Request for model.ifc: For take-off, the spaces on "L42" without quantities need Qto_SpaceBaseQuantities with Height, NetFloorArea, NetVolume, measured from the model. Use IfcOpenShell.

First a look at what the model holds.

```python
import ifcopenshell
import ifcopenshell.util.element
import ifcopenshell.util.unit

model = ifcopenshell.open("model.ifc")
print(model.schema)
for unit_type in ("LENGTHUNIT", "AREAUNIT", "VOLUMEUNIT"):
    print(unit_type, ifcopenshell.util.unit.calculate_unit_scale(model, unit_type))
storey = next(s for s in model.by_type("IfcBuildingStorey") if s.Name == "L42")
spaces = [e for e in ifcopenshell.util.element.get_decomposition(storey) if e.is_a("IfcSpace")]
for e in sorted(spaces, key=lambda e: e.id()):
    print(e.id(), e.is_a(), e.Name, list(ifcopenshell.util.element.get_psets(e, qtos_only=True)), sep=" | ")
```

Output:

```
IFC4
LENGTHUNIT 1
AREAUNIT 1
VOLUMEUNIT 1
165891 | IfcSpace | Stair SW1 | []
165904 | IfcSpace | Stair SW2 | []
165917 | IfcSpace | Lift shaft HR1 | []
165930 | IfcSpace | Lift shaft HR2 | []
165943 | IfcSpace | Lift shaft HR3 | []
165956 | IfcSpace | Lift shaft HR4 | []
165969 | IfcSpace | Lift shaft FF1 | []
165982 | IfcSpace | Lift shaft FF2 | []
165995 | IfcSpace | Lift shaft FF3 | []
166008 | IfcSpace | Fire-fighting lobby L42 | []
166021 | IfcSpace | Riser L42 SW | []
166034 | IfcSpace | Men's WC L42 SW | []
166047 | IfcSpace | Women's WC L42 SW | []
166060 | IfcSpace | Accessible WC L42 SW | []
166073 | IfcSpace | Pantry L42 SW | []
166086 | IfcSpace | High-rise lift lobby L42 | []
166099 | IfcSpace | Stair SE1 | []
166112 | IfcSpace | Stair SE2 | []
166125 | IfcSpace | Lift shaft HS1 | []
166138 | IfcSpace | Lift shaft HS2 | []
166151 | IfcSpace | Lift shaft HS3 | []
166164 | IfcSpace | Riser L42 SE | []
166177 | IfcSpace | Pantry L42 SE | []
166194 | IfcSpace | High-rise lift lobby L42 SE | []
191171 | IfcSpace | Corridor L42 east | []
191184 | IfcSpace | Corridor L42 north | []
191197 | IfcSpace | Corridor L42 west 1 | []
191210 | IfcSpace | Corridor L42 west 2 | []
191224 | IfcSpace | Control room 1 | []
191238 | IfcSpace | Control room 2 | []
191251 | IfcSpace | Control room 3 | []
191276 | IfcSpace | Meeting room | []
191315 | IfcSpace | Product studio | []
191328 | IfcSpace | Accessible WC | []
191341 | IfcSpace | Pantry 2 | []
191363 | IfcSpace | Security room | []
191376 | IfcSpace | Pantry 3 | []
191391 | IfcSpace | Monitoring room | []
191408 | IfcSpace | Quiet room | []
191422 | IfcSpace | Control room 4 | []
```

```python
import ifcopenshell
import ifcopenshell.api.pset
import ifcopenshell.geom
import ifcopenshell.util.element
import ifcopenshell.util.shape
import ifcopenshell.util.unit

model = ifcopenshell.open("model.ifc")
unit_scale = ifcopenshell.util.unit.calculate_unit_scale(model)
area_scale = ifcopenshell.util.unit.calculate_unit_scale(model, "AREAUNIT")
volume_scale = ifcopenshell.util.unit.calculate_unit_scale(model, "VOLUMEUNIT")
settings = ifcopenshell.geom.settings()

storey = next(s for s in model.by_type("IfcBuildingStorey") if s.Name == "L42")
spaces = [e for e in ifcopenshell.util.element.get_decomposition(storey) if e.is_a("IfcSpace")]

for e in sorted(spaces, key=lambda e: e.id()):
    if ifcopenshell.util.element.get_psets(e, qtos_only=True, should_inherit=False):
        continue
    # Geometry comes back in metres, in the element's own axes.
    shape = ifcopenshell.geom.create_shape(settings, e)
    values = {
        "Height": ifcopenshell.util.shape.get_z(shape.geometry) / unit_scale,
        "NetFloorArea": ifcopenshell.util.shape.get_footprint_area(shape.geometry) / area_scale,
        "NetVolume": ifcopenshell.util.shape.get_volume(shape.geometry) / volume_scale,
    }
    qto = ifcopenshell.api.pset.add_qto(model, product=e, name="Qto_SpaceBaseQuantities")
    ifcopenshell.api.pset.edit_qto(model, qto=qto, properties=values)
    print(e.id(), {k: round(v, 3) for k, v in values.items()})

model.write("model_rev.ifc")
```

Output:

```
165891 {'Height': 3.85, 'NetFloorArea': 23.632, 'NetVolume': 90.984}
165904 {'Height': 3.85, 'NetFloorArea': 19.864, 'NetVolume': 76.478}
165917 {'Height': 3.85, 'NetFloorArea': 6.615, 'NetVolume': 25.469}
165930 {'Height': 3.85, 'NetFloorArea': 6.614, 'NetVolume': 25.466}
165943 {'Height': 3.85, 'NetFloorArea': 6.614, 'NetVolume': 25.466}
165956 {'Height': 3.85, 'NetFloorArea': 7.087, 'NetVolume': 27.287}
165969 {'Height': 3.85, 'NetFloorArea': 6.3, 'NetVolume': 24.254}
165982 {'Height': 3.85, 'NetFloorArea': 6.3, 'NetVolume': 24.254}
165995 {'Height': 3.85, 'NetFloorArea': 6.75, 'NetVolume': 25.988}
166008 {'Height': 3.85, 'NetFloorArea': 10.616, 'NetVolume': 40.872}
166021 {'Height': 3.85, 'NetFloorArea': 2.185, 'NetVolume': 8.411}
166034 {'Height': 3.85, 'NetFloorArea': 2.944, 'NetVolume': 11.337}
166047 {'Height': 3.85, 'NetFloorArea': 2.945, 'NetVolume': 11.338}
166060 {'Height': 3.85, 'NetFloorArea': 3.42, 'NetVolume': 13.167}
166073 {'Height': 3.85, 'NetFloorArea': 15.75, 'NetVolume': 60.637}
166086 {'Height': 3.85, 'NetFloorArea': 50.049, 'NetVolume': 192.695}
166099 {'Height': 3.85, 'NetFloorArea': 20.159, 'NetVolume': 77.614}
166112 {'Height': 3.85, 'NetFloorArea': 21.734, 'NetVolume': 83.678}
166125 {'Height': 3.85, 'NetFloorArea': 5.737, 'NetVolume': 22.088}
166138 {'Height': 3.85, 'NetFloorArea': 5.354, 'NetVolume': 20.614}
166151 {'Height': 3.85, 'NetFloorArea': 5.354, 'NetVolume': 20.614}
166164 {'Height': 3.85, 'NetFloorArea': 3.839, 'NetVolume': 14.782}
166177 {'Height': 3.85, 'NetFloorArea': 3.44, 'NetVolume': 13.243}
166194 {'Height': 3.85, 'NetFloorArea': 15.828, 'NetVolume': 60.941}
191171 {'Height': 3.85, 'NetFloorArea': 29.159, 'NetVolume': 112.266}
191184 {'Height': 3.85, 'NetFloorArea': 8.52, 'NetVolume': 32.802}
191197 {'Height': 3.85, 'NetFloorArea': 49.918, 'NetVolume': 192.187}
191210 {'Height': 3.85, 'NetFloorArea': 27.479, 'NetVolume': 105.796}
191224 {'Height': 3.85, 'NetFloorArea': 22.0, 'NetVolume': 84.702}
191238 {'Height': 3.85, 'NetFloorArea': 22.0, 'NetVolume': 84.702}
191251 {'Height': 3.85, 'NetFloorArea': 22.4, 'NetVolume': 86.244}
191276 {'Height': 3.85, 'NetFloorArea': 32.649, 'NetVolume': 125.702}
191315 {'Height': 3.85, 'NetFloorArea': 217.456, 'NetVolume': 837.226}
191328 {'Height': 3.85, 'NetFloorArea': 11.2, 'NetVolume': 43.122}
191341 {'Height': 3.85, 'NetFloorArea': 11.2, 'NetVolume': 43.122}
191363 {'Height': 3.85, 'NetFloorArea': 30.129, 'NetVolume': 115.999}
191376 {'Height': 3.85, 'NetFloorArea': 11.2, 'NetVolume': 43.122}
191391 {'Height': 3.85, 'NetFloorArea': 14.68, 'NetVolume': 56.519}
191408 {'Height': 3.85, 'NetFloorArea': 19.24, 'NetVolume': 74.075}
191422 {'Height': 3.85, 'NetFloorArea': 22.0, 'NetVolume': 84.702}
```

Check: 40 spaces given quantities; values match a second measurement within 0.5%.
